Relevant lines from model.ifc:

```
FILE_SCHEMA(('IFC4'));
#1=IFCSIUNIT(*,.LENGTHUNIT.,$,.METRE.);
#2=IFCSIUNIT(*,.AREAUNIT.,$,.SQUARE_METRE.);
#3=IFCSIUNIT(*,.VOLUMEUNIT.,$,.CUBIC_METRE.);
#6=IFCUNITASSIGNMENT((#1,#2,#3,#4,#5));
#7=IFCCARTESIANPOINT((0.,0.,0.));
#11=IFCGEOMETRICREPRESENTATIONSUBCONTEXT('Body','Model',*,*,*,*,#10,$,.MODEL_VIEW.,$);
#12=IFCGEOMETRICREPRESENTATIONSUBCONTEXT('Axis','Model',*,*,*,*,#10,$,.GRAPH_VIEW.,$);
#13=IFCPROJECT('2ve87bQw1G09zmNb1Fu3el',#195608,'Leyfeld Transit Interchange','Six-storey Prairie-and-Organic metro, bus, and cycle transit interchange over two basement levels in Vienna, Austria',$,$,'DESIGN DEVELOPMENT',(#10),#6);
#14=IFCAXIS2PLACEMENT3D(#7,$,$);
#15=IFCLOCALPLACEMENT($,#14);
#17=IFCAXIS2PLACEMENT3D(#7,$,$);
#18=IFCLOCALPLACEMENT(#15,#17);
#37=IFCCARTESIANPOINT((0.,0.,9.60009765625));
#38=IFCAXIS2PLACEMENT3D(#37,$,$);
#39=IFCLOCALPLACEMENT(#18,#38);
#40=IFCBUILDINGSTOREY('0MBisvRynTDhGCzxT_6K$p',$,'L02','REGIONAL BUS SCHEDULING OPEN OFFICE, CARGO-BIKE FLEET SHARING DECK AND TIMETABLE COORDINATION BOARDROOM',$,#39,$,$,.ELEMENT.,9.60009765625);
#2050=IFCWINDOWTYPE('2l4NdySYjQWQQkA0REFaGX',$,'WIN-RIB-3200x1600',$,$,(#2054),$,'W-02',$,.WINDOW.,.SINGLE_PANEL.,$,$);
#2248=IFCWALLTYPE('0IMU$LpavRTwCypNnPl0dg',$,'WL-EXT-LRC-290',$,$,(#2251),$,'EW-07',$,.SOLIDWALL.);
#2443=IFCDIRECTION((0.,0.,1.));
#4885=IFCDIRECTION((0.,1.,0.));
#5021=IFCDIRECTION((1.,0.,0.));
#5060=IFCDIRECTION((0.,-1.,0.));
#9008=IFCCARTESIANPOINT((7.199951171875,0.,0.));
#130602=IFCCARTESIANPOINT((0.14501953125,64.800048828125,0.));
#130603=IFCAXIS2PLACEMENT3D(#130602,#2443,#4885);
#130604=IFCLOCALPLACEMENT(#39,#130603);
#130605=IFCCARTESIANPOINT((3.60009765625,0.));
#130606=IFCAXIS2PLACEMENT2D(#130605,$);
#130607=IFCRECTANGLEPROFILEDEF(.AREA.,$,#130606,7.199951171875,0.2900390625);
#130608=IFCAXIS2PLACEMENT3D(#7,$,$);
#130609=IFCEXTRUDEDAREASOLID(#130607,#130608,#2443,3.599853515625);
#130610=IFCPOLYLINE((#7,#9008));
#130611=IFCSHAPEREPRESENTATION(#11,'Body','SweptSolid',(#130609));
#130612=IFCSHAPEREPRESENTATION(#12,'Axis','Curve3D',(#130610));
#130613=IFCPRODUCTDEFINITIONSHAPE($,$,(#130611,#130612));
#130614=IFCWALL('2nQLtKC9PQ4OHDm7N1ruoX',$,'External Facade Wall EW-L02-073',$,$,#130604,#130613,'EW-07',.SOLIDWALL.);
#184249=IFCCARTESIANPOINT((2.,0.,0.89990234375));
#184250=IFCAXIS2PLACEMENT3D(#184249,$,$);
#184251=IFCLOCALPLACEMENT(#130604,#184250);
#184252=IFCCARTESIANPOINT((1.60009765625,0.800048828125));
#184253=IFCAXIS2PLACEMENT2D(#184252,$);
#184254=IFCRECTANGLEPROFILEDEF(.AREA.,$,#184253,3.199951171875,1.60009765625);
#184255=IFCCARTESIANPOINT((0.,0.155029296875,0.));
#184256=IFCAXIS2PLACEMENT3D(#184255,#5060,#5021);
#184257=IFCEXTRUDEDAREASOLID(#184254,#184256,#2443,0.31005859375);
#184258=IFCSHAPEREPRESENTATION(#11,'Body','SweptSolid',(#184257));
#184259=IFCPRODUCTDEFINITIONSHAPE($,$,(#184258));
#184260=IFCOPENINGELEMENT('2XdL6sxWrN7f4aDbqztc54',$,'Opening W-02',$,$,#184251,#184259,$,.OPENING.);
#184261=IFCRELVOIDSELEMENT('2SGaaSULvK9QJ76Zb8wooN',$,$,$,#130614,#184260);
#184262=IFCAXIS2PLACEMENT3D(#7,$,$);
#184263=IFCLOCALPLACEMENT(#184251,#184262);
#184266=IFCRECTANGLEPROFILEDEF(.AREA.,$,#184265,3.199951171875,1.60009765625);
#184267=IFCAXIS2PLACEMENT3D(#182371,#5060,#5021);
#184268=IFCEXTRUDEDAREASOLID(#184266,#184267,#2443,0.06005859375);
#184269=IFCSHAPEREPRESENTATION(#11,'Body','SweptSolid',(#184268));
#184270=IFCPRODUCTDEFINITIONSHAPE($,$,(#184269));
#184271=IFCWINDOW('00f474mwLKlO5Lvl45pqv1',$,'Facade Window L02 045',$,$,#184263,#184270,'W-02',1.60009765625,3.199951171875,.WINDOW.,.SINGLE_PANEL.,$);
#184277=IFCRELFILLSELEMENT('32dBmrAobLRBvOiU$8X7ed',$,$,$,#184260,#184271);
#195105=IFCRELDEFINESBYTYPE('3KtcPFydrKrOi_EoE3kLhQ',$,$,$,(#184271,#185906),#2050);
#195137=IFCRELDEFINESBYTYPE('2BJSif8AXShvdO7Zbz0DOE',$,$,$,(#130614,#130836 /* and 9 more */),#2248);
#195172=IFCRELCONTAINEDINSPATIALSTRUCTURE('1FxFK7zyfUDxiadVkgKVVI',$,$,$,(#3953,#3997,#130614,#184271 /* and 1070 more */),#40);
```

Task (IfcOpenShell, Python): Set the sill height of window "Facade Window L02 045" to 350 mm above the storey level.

```python
import numpy as np
import ifcopenshell
import ifcopenshell.api.geometry
import ifcopenshell.geom
import ifcopenshell.util.element
import ifcopenshell.util.placement
import ifcopenshell.util.shape
import ifcopenshell.util.unit

model = ifcopenshell.open("model.ifc")
unit_scale = ifcopenshell.util.unit.calculate_unit_scale(model)

window = model.by_guid("00f474mwLKlO5Lvl45pqv1")
opening = window.FillsVoids[0].RelatingOpeningElement
storey = ifcopenshell.util.element.get_container(window, ifc_class="IfcBuildingStorey")
level = ifcopenshell.util.placement.get_local_placement(storey.ObjectPlacement)[2, 3]

# The opening's origin need not be at the sill, so measure its lowest point.
shape = ifcopenshell.geom.create_shape(ifcopenshell.geom.settings(), opening)
bottom = ifcopenshell.util.shape.get_shape_bottom_elevation(shape, shape.geometry) / unit_scale
dz = level + 0.35 / unit_scale - bottom

shift = np.array([0.0, 0.0, dz])
# The window is placed relative to its opening, so it follows when the opening moves.
matrix = ifcopenshell.util.placement.get_local_placement(opening.ObjectPlacement)
matrix[:3, 3] += shift
ifcopenshell.api.geometry.edit_object_placement(
    model, product=opening, matrix=matrix, is_si=False, should_transform_children=True
)

print(f"moved by {dz * unit_scale:+.3f} m")

model.write("model_rev.ifc")
```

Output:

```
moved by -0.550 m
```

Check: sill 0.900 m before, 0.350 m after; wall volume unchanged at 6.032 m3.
